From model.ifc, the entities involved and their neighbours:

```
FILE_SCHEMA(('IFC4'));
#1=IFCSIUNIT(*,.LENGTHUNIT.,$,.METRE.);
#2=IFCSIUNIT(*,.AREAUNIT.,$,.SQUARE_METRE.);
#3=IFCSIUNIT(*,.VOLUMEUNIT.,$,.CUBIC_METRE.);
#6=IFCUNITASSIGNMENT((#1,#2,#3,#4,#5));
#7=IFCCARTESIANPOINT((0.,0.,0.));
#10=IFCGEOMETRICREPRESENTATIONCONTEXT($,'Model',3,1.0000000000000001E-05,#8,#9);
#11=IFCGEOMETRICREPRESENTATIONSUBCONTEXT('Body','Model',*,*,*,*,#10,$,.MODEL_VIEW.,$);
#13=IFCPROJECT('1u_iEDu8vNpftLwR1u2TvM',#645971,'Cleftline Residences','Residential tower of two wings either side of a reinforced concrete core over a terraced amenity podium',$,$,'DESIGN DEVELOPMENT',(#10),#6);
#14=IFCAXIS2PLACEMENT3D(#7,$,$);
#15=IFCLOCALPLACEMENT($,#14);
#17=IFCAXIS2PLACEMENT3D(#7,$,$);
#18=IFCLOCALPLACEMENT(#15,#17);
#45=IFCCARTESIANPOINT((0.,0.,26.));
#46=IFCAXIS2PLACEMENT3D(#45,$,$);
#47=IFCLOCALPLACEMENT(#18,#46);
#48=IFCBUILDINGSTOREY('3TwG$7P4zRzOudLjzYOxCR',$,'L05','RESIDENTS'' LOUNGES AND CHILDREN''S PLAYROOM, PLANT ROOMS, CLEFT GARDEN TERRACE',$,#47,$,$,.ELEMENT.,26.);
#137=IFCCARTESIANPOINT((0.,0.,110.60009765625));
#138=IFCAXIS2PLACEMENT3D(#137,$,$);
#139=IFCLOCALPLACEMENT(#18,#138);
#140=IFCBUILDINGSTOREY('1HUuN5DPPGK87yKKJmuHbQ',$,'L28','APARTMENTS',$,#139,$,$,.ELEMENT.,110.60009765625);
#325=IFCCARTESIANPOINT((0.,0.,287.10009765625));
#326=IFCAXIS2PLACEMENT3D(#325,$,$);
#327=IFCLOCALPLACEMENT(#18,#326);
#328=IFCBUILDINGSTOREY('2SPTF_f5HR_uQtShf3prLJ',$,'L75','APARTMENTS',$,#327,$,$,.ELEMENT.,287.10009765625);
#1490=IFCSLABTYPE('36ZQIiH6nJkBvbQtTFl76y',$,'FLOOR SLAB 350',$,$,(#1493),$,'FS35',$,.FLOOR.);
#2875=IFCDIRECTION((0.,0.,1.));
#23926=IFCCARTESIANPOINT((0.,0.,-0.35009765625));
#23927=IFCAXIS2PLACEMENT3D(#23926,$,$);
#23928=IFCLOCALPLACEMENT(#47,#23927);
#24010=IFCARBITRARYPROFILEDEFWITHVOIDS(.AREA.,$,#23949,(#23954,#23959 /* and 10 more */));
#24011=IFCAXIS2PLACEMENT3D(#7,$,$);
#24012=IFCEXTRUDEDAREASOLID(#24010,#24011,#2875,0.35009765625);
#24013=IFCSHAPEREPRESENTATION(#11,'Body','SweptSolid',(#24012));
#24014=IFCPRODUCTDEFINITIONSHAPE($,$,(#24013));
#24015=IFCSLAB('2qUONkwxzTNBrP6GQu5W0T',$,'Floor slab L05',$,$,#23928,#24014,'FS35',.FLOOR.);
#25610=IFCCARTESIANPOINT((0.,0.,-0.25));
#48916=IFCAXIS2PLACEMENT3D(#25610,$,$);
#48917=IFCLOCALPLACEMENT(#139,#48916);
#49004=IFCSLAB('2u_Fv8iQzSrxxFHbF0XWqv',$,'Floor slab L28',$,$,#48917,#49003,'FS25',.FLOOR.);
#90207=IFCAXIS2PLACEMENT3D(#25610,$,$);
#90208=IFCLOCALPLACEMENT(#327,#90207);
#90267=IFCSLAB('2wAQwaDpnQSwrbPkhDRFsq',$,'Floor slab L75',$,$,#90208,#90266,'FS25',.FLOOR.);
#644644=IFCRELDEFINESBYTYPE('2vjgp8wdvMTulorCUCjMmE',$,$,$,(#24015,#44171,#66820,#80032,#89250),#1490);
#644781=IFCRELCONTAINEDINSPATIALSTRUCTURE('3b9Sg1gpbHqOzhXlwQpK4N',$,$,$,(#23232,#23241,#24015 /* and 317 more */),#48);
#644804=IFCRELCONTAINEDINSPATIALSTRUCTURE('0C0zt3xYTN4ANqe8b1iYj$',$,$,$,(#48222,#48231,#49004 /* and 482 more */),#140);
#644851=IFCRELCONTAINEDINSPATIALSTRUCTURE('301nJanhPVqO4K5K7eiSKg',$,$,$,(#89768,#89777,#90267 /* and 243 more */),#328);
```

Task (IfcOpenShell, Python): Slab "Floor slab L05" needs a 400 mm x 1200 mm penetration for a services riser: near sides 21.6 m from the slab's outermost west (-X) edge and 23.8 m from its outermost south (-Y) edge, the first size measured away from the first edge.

```python
import numpy as np
import ifcopenshell
import ifcopenshell.api.feature
import ifcopenshell.api.geometry
import ifcopenshell.api.root
import ifcopenshell.geom
import ifcopenshell.util.placement
import ifcopenshell.util.representation
import ifcopenshell.util.shape
import ifcopenshell.util.unit

model = ifcopenshell.open("model.ifc")
unit_scale = ifcopenshell.util.unit.calculate_unit_scale(model)
settings = ifcopenshell.geom.settings()


def volume(element):
    """Net volume in cubic metres, openings subtracted."""
    shape = ifcopenshell.geom.create_shape(settings, element)
    return ifcopenshell.util.shape.get_volume(shape.geometry)


slab = model.by_guid("2qUONkwxzTNBrP6GQu5W0T")
before = volume(slab)

# Extent in the slab's own axes, in metres. The edges named are its -X and -Y sides.
slab_shape = ifcopenshell.geom.create_shape(settings, slab)
vertices = ifcopenshell.util.shape.get_vertices(slab_shape.geometry)
x_min, y_min, bottom = vertices.min(axis=0)
top = vertices[:, 2].max()

opening = ifcopenshell.api.root.create_entity(model, ifc_class="IfcOpeningElement", name="Services riser opening", predefined_type="OPENING")
context = ifcopenshell.util.representation.get_context(model, "Model", "Body", "MODEL_VIEW")
width, depth = 0.4, 1.2
outline = [(0.0, 0.0), (width, 0.0), (width, depth), (0.0, depth), (0.0, 0.0)]
# Overshoot both faces by 50 mm so the cut is clean.
shape = ifcopenshell.api.geometry.add_slab_representation(
    model, context=context, depth=top - bottom + 0.1, polyline=outline
)
ifcopenshell.api.geometry.assign_representation(model, product=opening, representation=shape)

matrix = ifcopenshell.util.placement.get_local_placement(slab.ObjectPlacement)
matrix[:, 3] = matrix @ np.append(np.array([x_min + 21.6, y_min + 23.8, bottom - 0.05]) / unit_scale, 1.0)
ifcopenshell.api.geometry.edit_object_placement(model, product=opening, matrix=matrix, is_si=False)
ifcopenshell.api.feature.add_feature(model, feature=opening, element=slab)

after = volume(slab)

print(f"slab volume {before:.3f} -> {after:.3f} m3")

model.write("model_rev.ifc")
```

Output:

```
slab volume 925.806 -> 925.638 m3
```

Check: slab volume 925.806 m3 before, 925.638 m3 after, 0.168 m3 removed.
